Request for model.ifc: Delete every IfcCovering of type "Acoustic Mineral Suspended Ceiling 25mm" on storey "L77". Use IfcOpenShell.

First a look at what the model holds.

```python
import ifcopenshell
import ifcopenshell.util.element

model = ifcopenshell.open("model.ifc")
print(model.schema)
storey = next(s for s in model.by_type("IfcBuildingStorey") if s.Name == "L77")
coverings = [e for e in ifcopenshell.util.element.get_decomposition(storey) if e.is_a("IfcCovering")]
seen = {}
for e in coverings:
    element_type = ifcopenshell.util.element.get_type(e)
    name = element_type.Name if element_type not in (None, e) else None
    seen[name] = seen.get(name, 0) + 1
for name, count in sorted(seen.items(), key=str):
    print(count, "x", name)
```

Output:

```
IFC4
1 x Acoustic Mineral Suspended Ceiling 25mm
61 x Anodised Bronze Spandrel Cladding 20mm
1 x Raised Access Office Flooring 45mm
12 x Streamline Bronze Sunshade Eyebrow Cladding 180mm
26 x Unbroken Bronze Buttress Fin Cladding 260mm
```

```python
import ifcopenshell
import ifcopenshell.api.root
import ifcopenshell.util.element

model = ifcopenshell.open("model.ifc")

storey = next(s for s in model.by_type("IfcBuildingStorey") if s.Name == "L77")
coverings = [e for e in ifcopenshell.util.element.get_decomposition(storey) if e.is_a("IfcCovering")]
targets = [e for e in coverings if (t := ifcopenshell.util.element.get_type(e)) not in (None, e) and t.Name == "Acoustic Mineral Suspended Ceiling 25mm"]

for e in targets:
    ifcopenshell.api.root.remove_product(model, product=e)
print(len(targets), "removed")

model.write("model-out.ifc")
```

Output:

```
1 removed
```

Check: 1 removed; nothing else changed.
